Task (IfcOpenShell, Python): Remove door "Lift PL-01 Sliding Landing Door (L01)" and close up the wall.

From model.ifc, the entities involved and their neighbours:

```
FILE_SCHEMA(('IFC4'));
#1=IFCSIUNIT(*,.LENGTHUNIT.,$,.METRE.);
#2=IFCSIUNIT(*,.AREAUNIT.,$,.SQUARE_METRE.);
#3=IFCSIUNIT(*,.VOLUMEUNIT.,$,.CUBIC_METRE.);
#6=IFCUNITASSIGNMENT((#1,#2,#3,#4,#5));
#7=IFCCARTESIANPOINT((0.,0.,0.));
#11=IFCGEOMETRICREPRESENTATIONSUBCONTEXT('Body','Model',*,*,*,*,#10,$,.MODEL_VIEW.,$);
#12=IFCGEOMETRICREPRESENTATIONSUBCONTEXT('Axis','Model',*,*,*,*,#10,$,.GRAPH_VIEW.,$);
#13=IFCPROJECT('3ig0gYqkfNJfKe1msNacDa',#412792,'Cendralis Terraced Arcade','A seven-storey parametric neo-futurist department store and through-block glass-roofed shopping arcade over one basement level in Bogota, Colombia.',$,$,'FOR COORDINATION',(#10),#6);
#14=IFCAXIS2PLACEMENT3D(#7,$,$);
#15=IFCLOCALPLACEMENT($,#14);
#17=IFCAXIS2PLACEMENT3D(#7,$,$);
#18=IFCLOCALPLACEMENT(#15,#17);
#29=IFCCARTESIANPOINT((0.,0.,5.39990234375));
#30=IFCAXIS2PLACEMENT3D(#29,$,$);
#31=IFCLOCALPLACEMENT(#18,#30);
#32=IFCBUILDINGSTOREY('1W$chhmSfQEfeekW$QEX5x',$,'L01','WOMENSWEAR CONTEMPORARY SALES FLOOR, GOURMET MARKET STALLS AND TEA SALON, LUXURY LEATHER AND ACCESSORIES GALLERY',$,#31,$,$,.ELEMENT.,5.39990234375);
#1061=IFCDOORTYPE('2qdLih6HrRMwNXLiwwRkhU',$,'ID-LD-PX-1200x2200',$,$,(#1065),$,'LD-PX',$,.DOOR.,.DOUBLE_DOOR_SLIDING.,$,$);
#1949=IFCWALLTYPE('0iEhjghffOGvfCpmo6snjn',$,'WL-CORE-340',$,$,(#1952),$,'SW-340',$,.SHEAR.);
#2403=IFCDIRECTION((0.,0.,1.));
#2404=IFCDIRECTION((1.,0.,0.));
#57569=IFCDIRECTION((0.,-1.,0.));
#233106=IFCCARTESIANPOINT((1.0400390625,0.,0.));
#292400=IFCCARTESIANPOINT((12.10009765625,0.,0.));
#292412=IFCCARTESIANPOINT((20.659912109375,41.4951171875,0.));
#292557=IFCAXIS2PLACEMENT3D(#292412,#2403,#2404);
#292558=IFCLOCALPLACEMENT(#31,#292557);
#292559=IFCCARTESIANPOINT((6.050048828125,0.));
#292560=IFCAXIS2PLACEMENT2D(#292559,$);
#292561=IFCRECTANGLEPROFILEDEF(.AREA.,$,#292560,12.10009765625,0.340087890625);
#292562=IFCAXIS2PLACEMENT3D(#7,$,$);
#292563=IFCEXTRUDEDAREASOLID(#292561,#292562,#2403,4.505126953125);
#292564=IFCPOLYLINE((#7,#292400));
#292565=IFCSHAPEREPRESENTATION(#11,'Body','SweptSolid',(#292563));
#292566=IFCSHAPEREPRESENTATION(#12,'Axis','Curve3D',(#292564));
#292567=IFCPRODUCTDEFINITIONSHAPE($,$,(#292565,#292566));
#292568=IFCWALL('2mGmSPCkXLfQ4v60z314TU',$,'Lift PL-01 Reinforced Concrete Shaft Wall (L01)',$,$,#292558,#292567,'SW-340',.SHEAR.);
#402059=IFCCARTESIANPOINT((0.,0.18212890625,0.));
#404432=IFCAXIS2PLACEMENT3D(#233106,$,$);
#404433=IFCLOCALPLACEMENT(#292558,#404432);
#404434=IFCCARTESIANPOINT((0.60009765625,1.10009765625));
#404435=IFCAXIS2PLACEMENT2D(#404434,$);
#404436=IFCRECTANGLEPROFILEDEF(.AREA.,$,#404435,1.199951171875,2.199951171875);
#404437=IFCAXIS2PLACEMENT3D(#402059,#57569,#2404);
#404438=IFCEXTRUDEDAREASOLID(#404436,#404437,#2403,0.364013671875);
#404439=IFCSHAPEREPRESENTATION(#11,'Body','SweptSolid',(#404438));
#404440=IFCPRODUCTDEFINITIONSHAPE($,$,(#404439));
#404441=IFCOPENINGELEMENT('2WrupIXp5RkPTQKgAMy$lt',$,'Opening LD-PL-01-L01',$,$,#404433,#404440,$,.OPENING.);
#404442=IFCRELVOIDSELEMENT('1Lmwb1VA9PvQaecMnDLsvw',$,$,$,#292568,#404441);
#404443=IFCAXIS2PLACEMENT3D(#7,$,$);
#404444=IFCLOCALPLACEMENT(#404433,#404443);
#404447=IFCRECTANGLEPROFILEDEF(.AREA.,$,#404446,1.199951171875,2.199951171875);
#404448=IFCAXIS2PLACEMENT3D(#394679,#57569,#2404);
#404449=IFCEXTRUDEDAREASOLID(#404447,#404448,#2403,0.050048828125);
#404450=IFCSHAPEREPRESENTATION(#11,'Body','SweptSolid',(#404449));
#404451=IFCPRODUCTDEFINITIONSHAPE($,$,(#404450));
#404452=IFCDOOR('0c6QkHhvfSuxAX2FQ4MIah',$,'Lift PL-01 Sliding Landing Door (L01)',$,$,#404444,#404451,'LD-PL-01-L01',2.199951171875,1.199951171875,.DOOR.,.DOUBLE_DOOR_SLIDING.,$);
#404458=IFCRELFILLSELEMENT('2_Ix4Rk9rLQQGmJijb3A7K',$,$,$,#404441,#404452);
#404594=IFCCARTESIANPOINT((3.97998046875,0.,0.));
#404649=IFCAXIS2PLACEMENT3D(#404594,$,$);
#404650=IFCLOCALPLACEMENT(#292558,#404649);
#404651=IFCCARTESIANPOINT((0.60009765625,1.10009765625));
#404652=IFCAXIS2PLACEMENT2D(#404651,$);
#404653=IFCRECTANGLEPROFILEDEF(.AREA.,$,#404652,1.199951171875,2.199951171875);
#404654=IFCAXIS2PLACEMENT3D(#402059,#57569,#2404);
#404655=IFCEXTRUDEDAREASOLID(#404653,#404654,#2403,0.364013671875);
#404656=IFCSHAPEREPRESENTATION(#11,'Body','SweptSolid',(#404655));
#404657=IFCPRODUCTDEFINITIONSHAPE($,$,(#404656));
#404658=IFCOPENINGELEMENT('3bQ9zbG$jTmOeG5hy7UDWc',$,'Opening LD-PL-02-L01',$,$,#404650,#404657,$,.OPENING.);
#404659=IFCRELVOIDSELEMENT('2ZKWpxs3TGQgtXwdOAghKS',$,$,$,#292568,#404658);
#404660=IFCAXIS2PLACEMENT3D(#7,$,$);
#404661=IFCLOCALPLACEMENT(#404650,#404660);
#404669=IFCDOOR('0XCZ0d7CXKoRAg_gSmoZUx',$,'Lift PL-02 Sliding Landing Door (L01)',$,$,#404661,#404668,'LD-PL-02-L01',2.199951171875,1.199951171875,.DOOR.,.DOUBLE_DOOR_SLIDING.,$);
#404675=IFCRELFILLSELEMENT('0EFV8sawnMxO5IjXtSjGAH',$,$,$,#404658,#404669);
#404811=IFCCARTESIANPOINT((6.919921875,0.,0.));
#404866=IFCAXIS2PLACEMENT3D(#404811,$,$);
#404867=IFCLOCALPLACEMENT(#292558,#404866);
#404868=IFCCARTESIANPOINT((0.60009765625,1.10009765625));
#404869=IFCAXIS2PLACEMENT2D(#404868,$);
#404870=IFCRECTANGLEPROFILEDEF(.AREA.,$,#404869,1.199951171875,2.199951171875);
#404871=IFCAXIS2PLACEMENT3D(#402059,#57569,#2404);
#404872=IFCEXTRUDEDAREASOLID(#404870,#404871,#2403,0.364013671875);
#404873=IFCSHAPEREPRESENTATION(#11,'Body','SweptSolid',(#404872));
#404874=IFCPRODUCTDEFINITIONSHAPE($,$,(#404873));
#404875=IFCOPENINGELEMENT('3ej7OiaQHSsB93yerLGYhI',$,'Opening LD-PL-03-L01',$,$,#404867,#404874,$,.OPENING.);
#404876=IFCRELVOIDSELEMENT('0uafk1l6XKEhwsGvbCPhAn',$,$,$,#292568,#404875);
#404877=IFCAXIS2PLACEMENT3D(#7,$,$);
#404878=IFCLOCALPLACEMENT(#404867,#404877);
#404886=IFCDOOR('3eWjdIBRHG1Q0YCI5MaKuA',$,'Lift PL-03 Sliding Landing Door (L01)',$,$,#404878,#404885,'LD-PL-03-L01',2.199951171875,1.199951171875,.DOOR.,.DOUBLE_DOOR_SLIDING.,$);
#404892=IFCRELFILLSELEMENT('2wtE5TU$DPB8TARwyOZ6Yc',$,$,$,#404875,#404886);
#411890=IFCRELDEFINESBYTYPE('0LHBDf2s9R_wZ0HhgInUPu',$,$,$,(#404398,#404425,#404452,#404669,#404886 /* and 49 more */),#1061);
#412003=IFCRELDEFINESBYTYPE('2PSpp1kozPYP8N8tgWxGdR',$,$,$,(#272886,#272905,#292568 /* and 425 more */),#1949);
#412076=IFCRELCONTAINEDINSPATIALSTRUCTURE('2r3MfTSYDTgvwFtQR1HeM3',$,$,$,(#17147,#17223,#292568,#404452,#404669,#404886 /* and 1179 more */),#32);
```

```python
import ifcopenshell
import ifcopenshell.api.feature
import ifcopenshell.api.root
import ifcopenshell.geom
import ifcopenshell.util.shape

model = ifcopenshell.open("model.ifc")
settings = ifcopenshell.geom.settings()


def volume(element):
    """Net volume in cubic metres, openings subtracted."""
    shape = ifcopenshell.geom.create_shape(settings, element)
    return ifcopenshell.util.shape.get_volume(shape.geometry)


door = model.by_guid("0c6QkHhvfSuxAX2FQ4MIah")
opening = door.FillsVoids[0].RelatingOpeningElement
wall = opening.VoidsElements[0].RelatingBuildingElement
before = volume(wall)

ifcopenshell.api.root.remove_product(model, product=door)
ifcopenshell.api.feature.remove_feature(model, feature=opening)

after = volume(wall)

print(f"wall volume {before:.3f} -> {after:.3f} m3")

model.write("model_v2.ifc")
```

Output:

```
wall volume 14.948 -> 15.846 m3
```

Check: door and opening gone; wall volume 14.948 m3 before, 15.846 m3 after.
